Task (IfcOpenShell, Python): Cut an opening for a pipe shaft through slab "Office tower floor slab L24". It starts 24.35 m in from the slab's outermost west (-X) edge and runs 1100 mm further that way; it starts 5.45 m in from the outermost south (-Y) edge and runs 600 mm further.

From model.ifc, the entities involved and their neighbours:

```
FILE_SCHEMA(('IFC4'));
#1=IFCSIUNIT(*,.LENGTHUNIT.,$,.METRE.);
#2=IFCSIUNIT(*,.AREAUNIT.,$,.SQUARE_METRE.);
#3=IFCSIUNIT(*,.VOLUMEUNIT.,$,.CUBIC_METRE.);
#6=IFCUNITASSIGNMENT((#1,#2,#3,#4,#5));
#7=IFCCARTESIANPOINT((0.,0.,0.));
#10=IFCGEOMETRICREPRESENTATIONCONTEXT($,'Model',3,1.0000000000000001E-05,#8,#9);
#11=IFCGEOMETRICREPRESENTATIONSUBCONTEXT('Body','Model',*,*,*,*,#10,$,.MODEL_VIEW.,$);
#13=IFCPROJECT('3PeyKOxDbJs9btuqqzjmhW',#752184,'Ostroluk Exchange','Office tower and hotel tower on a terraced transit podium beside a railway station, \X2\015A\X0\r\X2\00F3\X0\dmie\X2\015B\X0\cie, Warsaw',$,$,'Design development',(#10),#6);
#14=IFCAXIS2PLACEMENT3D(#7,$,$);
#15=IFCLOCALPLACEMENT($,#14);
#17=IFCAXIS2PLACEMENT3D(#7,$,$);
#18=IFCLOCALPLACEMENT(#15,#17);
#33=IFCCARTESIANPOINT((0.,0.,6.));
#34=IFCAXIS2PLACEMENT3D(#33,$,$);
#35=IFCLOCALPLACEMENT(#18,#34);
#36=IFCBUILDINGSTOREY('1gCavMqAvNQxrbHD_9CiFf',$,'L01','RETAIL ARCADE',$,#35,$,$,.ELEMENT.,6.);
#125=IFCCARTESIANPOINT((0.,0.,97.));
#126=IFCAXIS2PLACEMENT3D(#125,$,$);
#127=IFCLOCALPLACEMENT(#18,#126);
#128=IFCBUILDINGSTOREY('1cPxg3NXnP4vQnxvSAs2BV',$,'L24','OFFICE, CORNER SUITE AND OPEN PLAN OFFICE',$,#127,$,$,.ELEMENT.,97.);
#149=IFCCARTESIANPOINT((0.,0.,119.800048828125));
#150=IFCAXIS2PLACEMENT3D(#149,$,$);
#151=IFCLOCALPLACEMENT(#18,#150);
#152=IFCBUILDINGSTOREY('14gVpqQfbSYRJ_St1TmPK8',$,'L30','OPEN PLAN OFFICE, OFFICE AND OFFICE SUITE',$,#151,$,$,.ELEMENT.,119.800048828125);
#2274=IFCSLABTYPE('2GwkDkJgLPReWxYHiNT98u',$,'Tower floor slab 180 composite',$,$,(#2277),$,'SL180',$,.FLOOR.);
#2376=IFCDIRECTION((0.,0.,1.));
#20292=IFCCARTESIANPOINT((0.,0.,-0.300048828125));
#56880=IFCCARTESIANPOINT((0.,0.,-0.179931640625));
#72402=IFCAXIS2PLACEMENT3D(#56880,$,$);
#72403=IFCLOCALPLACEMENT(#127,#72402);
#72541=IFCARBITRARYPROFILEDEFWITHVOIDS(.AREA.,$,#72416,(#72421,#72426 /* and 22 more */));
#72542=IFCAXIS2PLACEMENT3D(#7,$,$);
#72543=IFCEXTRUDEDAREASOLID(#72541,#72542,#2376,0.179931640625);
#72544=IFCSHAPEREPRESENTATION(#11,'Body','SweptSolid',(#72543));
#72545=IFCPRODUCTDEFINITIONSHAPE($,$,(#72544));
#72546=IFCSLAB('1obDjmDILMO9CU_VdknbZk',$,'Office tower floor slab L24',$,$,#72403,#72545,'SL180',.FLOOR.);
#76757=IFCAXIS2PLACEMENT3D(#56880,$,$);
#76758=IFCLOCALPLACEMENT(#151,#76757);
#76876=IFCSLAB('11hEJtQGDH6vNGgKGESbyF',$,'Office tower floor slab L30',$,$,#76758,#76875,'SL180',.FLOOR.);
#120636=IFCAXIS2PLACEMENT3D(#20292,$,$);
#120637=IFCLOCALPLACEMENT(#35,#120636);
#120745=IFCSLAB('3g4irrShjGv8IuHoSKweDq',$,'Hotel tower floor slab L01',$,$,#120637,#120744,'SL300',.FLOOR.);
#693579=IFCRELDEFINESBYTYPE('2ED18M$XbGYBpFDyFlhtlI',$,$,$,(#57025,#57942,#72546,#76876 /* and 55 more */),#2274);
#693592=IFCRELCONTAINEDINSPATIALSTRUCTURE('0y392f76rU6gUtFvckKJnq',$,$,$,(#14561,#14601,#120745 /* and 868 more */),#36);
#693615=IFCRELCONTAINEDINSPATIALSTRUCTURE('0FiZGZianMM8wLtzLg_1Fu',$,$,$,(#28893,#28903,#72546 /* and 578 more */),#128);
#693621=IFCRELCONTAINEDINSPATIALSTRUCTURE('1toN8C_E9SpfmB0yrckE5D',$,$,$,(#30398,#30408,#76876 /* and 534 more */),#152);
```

```python
import numpy as np
import ifcopenshell
import ifcopenshell.api.feature
import ifcopenshell.api.geometry
import ifcopenshell.api.root
import ifcopenshell.geom
import ifcopenshell.util.placement
import ifcopenshell.util.representation
import ifcopenshell.util.shape
import ifcopenshell.util.unit

model = ifcopenshell.open("model.ifc")
unit_scale = ifcopenshell.util.unit.calculate_unit_scale(model)
settings = ifcopenshell.geom.settings()


def volume(element):
    """Net volume in cubic metres, openings subtracted."""
    shape = ifcopenshell.geom.create_shape(settings, element)
    return ifcopenshell.util.shape.get_volume(shape.geometry)


slab = model.by_guid("1obDjmDILMO9CU_VdknbZk")
before = volume(slab)

# Extent in the slab's own axes, in metres. The edges named are its -X and -Y sides.
slab_shape = ifcopenshell.geom.create_shape(settings, slab)
vertices = ifcopenshell.util.shape.get_vertices(slab_shape.geometry)
x_min, y_min, bottom = vertices.min(axis=0)
top = vertices[:, 2].max()

opening = ifcopenshell.api.root.create_entity(model, ifc_class="IfcOpeningElement", name="Pipe shaft opening", predefined_type="OPENING")
context = ifcopenshell.util.representation.get_context(model, "Model", "Body", "MODEL_VIEW")
width, depth = 1.1, 0.6
outline = [(0.0, 0.0), (width, 0.0), (width, depth), (0.0, depth), (0.0, 0.0)]
# Overshoot both faces by 50 mm so the cut is clean.
shape = ifcopenshell.api.geometry.add_slab_representation(
    model, context=context, depth=top - bottom + 0.1, polyline=outline
)
ifcopenshell.api.geometry.assign_representation(model, product=opening, representation=shape)

matrix = ifcopenshell.util.placement.get_local_placement(slab.ObjectPlacement)
matrix[:, 3] = matrix @ np.append(np.array([x_min + 24.35, y_min + 5.45, bottom - 0.05]) / unit_scale, 1.0)
ifcopenshell.api.geometry.edit_object_placement(model, product=opening, matrix=matrix, is_si=False)
ifcopenshell.api.feature.add_feature(model, feature=opening, element=slab)

after = volume(slab)

print(f"slab volume {before:.3f} -> {after:.3f} m3")

model.write("model_rev.ifc")
```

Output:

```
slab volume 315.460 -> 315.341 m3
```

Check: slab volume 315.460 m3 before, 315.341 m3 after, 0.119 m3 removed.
